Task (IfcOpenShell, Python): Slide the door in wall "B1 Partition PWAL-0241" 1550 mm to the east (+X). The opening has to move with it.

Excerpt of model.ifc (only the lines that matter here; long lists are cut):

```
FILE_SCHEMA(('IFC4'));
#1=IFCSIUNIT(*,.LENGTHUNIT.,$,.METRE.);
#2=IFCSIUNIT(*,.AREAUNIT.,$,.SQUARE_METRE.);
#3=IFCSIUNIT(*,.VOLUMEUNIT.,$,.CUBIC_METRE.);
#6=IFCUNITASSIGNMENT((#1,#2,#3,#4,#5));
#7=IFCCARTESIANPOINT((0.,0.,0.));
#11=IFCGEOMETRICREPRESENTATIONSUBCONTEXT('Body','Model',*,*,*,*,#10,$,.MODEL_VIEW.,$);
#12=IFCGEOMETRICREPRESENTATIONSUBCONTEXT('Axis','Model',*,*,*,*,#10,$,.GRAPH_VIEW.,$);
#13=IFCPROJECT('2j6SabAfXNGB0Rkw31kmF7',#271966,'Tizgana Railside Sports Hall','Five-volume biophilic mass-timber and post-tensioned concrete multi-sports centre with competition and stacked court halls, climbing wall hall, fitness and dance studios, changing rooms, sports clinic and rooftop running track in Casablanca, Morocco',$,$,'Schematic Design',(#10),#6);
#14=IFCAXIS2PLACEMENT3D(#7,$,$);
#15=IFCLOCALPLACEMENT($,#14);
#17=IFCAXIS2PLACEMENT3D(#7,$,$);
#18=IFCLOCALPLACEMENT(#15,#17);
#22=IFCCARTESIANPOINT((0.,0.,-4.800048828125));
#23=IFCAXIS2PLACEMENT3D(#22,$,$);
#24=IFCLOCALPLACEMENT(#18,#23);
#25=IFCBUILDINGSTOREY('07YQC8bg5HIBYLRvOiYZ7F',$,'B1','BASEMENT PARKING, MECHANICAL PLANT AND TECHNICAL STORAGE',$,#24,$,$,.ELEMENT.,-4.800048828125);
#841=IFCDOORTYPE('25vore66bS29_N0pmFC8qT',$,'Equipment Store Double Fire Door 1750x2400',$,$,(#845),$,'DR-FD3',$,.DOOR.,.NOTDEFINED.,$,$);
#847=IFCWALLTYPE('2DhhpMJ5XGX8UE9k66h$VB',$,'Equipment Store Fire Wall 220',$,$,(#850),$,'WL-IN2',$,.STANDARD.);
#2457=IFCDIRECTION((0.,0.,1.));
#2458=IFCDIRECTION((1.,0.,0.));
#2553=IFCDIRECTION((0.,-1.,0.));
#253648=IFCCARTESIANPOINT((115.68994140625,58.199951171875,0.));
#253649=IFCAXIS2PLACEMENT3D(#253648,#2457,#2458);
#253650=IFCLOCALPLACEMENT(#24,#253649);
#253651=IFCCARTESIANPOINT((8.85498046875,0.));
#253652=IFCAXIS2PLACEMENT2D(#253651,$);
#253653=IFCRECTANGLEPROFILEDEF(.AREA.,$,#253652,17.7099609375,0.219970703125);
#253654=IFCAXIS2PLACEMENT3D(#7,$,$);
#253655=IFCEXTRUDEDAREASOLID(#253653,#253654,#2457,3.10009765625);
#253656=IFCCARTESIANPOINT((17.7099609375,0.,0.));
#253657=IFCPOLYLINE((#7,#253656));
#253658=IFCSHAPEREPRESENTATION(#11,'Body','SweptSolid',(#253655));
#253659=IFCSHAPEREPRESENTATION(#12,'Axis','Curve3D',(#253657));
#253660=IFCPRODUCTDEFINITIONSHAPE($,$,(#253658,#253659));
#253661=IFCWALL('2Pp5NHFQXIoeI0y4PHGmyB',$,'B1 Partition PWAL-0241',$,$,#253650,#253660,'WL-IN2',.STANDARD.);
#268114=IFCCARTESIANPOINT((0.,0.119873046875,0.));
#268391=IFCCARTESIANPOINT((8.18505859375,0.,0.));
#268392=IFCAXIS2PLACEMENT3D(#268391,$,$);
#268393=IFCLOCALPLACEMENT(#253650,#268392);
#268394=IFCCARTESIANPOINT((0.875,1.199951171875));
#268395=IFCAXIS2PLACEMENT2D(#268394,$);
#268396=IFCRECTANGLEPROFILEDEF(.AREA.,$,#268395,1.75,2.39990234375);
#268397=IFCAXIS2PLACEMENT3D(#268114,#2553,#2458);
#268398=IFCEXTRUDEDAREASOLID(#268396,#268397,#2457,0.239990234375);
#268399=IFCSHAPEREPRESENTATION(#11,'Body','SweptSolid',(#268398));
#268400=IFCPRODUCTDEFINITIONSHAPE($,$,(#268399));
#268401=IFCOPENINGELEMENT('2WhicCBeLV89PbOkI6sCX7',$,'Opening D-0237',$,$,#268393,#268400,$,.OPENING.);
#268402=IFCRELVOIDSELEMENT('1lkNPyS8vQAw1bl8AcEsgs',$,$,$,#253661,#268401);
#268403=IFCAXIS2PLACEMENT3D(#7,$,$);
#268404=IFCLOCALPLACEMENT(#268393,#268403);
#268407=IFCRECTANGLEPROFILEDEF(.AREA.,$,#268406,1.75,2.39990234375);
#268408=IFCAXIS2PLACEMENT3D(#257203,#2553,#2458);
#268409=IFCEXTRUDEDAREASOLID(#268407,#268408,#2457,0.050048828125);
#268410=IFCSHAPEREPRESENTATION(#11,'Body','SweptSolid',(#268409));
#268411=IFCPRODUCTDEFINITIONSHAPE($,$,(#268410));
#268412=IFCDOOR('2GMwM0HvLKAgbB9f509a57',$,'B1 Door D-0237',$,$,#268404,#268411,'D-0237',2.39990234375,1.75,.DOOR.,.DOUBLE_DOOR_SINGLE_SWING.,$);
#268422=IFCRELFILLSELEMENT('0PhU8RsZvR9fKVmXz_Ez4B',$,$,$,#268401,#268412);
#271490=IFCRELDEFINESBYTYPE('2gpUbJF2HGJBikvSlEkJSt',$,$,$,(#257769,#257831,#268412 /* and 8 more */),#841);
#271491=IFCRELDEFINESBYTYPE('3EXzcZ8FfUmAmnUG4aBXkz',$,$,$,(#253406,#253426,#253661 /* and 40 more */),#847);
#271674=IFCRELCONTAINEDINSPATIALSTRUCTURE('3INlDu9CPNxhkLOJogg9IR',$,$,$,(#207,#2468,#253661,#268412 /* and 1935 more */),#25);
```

```python
import ifcopenshell
import ifcopenshell.api.geometry
import ifcopenshell.util.placement
import ifcopenshell.util.unit

model = ifcopenshell.open("model.ifc")
unit_scale = ifcopenshell.util.unit.calculate_unit_scale(model)

door = model.by_id(268412)
opening = door.FillsVoids[0].RelatingOpeningElement
wall = opening.VoidsElements[0].RelatingBuildingElement

wall_matrix = ifcopenshell.util.placement.get_local_placement(wall.ObjectPlacement)
shift = wall_matrix[:3, 0] * 1.55 / unit_scale
before = ifcopenshell.util.placement.get_local_placement(door.ObjectPlacement)[:3, 3].copy()

# The door is placed relative to its opening, so it follows when the opening moves.
matrix = ifcopenshell.util.placement.get_local_placement(opening.ObjectPlacement)
matrix[:3, 3] += shift
ifcopenshell.api.geometry.edit_object_placement(
    model, product=opening, matrix=matrix, is_si=False, should_transform_children=True
)

after = ifcopenshell.util.placement.get_local_placement(door.ObjectPlacement)[:3, 3]
print("door moved by", (after - before).round(3) + 0.0)

model.write("model_rev.ifc")
```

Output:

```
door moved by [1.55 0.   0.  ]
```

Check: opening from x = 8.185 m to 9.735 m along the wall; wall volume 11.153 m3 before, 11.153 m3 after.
